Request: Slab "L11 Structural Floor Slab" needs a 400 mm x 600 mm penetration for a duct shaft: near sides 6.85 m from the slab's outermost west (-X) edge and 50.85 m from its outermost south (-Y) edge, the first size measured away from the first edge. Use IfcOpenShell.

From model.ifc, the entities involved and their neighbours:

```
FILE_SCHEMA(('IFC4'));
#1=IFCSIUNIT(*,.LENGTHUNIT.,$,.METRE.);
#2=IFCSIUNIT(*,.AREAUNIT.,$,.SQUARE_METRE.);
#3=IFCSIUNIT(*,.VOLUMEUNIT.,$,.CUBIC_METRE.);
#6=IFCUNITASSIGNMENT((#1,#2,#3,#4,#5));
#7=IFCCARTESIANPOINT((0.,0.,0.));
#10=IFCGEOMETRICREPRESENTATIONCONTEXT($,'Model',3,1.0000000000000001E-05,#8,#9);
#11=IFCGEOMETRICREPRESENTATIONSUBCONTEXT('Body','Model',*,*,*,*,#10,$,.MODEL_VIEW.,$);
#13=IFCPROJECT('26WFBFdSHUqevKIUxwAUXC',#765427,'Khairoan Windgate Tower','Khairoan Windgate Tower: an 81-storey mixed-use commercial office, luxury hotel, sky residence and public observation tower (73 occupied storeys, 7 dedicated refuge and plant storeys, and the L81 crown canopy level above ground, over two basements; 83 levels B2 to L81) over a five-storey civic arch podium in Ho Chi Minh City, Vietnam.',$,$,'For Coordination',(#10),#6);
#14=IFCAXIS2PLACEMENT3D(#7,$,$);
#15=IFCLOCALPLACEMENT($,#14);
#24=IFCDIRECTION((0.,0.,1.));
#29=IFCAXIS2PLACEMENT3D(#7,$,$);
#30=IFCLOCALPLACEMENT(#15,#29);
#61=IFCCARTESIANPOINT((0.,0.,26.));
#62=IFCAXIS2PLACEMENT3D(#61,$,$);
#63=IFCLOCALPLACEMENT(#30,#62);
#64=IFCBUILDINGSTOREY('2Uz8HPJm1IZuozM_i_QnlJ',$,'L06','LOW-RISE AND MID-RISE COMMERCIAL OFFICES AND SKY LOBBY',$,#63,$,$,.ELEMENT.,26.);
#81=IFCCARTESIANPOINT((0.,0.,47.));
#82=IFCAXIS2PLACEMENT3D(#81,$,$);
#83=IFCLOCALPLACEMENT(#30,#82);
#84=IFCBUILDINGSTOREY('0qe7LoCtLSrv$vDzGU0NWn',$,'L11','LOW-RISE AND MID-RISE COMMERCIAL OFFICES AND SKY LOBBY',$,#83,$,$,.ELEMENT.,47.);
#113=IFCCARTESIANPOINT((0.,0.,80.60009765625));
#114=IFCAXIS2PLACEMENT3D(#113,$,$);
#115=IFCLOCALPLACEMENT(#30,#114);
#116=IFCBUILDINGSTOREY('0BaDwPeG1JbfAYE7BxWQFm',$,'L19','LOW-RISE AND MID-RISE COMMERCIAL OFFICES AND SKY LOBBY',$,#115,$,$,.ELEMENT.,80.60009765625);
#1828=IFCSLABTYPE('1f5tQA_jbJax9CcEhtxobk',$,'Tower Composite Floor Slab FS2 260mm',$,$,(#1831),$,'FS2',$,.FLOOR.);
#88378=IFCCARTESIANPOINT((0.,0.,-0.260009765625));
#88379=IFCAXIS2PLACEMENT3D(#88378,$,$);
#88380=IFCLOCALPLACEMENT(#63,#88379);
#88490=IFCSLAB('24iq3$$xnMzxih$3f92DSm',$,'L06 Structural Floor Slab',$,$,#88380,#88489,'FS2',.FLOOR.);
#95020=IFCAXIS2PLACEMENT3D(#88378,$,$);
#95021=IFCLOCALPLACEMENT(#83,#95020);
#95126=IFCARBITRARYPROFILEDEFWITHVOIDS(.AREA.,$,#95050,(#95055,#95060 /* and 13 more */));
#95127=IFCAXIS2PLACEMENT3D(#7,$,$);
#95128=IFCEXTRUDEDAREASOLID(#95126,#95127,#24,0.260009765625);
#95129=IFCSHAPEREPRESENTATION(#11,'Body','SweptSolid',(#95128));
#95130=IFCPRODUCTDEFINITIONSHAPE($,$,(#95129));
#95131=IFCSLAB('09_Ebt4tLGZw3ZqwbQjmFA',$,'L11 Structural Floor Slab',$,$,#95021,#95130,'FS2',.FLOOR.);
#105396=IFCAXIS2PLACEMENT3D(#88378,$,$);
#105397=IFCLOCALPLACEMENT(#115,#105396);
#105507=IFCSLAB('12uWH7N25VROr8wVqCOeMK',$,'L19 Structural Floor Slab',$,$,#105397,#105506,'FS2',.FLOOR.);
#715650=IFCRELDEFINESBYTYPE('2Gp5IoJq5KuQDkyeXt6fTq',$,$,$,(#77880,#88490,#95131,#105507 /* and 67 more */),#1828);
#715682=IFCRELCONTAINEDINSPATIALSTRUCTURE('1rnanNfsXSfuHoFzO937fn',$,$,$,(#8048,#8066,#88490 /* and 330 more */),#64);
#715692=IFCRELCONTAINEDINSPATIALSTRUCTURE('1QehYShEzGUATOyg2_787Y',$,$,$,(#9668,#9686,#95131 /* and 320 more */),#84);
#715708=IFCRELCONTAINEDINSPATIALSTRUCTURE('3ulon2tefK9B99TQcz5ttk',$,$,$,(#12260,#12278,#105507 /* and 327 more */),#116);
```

```python
import numpy as np
import ifcopenshell
import ifcopenshell.api.feature
import ifcopenshell.api.geometry
import ifcopenshell.api.root
import ifcopenshell.geom
import ifcopenshell.util.placement
import ifcopenshell.util.representation
import ifcopenshell.util.shape
import ifcopenshell.util.unit

model = ifcopenshell.open("model.ifc")
unit_scale = ifcopenshell.util.unit.calculate_unit_scale(model)
settings = ifcopenshell.geom.settings()


def volume(element):
    """Net volume in cubic metres, openings subtracted."""
    shape = ifcopenshell.geom.create_shape(settings, element)
    return ifcopenshell.util.shape.get_volume(shape.geometry)


slab = model.by_guid("09_Ebt4tLGZw3ZqwbQjmFA")
before = volume(slab)

# Extent in the slab's own axes, in metres. The edges named are its -X and -Y sides.
slab_shape = ifcopenshell.geom.create_shape(settings, slab)
vertices = ifcopenshell.util.shape.get_vertices(slab_shape.geometry)
x_min, y_min, bottom = vertices.min(axis=0)
top = vertices[:, 2].max()

opening = ifcopenshell.api.root.create_entity(model, ifc_class="IfcOpeningElement", name="Duct shaft opening", predefined_type="OPENING")
context = ifcopenshell.util.representation.get_context(model, "Model", "Body", "MODEL_VIEW")
width, depth = 0.4, 0.6
outline = [(0.0, 0.0), (width, 0.0), (width, depth), (0.0, depth), (0.0, 0.0)]
# Overshoot both faces by 50 mm so the cut is clean.
shape = ifcopenshell.api.geometry.add_slab_representation(
    model, context=context, depth=top - bottom + 0.1, polyline=outline
)
ifcopenshell.api.geometry.assign_representation(model, product=opening, representation=shape)

matrix = ifcopenshell.util.placement.get_local_placement(slab.ObjectPlacement)
matrix[:, 3] = matrix @ np.append(np.array([x_min + 6.85, y_min + 50.85, bottom - 0.05]) / unit_scale, 1.0)
ifcopenshell.api.geometry.edit_object_placement(model, product=opening, matrix=matrix, is_si=False)
ifcopenshell.api.feature.add_feature(model, feature=opening, element=slab)

after = volume(slab)

print(f"slab volume {before:.3f} -> {after:.3f} m3")

model.write("model_edited.ifc")
```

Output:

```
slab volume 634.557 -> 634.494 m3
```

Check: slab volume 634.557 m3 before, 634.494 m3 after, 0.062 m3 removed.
